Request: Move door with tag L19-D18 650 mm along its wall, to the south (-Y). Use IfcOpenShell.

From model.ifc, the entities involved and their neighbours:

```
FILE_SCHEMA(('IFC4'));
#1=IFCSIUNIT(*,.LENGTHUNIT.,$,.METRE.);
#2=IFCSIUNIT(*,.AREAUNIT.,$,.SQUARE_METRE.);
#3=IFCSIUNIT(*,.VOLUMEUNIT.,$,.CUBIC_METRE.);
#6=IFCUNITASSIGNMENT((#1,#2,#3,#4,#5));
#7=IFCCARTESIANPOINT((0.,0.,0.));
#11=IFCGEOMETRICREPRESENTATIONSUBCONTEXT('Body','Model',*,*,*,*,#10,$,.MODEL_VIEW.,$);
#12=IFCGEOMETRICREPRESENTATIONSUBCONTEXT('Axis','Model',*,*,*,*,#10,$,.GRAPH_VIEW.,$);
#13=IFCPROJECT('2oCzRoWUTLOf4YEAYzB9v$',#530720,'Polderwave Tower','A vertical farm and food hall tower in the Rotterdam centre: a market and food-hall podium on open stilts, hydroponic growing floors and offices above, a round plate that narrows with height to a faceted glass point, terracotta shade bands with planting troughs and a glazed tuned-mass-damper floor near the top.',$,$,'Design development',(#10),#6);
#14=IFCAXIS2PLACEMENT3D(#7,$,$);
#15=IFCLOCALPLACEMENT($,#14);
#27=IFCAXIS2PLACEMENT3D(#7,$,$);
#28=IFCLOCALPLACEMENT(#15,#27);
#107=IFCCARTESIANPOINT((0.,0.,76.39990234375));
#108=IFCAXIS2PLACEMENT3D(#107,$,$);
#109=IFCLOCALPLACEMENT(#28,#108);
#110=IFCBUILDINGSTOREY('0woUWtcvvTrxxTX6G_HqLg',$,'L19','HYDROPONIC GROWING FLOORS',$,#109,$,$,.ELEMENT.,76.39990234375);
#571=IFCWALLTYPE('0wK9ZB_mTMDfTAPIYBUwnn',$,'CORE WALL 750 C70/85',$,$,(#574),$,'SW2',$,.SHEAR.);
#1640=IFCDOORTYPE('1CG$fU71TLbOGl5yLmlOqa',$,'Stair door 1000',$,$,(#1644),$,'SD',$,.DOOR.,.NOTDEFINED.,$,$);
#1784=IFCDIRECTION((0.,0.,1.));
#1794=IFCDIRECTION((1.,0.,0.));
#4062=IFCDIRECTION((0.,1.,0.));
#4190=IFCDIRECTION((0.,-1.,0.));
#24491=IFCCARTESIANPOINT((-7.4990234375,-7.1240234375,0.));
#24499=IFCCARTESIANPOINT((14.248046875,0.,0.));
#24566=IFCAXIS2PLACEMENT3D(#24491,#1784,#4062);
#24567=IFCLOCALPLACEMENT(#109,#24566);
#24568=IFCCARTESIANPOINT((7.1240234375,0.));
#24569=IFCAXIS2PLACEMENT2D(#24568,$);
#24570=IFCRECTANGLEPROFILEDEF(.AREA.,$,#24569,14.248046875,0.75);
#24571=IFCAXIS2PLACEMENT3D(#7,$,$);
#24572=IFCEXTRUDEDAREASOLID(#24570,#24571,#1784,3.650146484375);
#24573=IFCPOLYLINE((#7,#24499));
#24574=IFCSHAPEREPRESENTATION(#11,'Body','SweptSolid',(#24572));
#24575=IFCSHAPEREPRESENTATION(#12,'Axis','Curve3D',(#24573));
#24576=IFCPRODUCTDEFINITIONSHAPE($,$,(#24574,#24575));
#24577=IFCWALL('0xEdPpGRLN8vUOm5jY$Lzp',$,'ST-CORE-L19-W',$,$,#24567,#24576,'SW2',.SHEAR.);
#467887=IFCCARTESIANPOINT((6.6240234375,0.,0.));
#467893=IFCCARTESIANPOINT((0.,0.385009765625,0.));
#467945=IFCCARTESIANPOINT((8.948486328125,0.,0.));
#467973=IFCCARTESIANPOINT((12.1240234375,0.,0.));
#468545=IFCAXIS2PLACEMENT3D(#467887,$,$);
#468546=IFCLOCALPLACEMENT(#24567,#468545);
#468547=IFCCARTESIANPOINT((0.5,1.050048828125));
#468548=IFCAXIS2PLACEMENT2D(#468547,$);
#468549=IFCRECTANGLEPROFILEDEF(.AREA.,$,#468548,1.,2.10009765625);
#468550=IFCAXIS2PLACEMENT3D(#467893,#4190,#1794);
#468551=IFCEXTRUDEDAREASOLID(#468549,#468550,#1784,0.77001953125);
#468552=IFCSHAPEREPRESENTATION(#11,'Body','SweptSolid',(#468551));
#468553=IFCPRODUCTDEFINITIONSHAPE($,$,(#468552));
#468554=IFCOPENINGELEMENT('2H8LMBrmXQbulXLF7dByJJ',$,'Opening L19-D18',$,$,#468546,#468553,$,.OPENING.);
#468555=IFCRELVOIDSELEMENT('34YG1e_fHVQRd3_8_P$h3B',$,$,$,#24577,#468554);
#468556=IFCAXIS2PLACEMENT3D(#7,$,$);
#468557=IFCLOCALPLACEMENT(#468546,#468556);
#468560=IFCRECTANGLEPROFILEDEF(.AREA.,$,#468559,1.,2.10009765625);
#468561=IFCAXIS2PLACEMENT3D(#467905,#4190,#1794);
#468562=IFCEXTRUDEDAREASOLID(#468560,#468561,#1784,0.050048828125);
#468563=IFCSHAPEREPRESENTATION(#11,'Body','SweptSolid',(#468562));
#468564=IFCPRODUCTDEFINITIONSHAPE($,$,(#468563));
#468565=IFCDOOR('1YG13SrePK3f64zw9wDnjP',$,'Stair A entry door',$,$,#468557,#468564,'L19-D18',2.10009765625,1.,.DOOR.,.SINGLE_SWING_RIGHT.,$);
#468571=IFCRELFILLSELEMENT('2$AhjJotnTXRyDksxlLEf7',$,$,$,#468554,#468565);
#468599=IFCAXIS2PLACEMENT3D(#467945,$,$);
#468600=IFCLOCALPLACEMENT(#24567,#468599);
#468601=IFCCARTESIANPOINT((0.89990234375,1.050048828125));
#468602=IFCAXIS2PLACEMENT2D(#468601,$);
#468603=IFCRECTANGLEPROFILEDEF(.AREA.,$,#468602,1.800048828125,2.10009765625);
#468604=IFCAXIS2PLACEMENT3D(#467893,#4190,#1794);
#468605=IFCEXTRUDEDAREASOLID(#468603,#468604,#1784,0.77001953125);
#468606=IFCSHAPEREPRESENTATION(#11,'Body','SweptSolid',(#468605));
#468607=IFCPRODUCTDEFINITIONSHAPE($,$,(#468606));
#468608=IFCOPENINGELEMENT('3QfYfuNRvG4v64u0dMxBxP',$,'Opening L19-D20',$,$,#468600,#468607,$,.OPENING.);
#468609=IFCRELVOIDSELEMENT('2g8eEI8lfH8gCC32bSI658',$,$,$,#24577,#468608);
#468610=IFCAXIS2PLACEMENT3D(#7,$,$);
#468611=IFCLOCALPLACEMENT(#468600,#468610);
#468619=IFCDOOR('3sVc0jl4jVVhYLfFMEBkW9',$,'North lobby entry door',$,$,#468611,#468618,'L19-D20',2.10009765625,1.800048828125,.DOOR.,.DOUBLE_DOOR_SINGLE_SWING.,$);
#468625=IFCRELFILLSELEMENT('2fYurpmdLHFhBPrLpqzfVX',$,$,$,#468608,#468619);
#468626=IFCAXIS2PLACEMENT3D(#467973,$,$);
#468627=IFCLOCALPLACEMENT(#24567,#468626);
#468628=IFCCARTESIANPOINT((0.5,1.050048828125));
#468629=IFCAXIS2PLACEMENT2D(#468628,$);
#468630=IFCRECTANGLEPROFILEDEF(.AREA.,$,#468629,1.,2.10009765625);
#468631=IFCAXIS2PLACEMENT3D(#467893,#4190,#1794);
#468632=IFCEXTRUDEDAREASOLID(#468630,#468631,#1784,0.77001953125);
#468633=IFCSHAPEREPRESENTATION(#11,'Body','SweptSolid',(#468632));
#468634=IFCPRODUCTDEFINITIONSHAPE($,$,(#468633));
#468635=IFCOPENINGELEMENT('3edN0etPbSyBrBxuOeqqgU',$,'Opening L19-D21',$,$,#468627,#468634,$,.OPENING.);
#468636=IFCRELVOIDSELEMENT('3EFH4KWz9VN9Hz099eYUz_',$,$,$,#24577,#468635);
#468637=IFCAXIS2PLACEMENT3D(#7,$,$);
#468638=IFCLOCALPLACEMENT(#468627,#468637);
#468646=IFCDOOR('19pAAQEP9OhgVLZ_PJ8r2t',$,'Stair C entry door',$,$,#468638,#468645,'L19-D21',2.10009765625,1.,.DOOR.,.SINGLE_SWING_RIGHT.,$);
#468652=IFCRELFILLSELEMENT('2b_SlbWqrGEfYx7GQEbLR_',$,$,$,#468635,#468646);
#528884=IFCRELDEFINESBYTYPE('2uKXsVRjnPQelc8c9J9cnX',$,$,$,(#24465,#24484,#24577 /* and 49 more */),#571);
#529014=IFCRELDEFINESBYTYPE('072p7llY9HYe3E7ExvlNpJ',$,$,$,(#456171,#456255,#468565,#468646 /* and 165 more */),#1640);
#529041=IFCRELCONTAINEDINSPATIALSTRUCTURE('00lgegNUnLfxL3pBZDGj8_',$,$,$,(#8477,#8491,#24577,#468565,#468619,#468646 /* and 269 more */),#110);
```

```python
import ifcopenshell
import ifcopenshell.api.geometry
import ifcopenshell.util.placement
import ifcopenshell.util.unit

model = ifcopenshell.open("model.ifc")
unit_scale = ifcopenshell.util.unit.calculate_unit_scale(model)

door = model.by_guid("1YG13SrePK3f64zw9wDnjP")
opening = door.FillsVoids[0].RelatingOpeningElement
wall = opening.VoidsElements[0].RelatingBuildingElement

wall_matrix = ifcopenshell.util.placement.get_local_placement(wall.ObjectPlacement)
shift = wall_matrix[:3, 0] * -0.65 / unit_scale
before = ifcopenshell.util.placement.get_local_placement(door.ObjectPlacement)[:3, 3].copy()

# The door is placed relative to its opening, so it follows when the opening moves.
matrix = ifcopenshell.util.placement.get_local_placement(opening.ObjectPlacement)
matrix[:3, 3] += shift
ifcopenshell.api.geometry.edit_object_placement(
    model, product=opening, matrix=matrix, is_si=False, should_transform_children=True
)

after = ifcopenshell.util.placement.get_local_placement(door.ObjectPlacement)[:3, 3]
print("door moved by", (after - before).round(3) + 0.0)

model.write("model_rev.ifc")
```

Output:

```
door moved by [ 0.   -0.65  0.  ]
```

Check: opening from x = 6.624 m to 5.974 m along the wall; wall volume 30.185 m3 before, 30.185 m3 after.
